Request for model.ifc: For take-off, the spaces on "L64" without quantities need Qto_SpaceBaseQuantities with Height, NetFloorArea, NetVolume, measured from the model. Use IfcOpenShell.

First a look at what the model holds.

```python
import ifcopenshell
import ifcopenshell.util.element
import ifcopenshell.util.unit

model = ifcopenshell.open("model.ifc")
print(model.schema)
for unit_type in ("LENGTHUNIT", "AREAUNIT", "VOLUMEUNIT"):
    print(unit_type, ifcopenshell.util.unit.calculate_unit_scale(model, unit_type))
storey = next(s for s in model.by_type("IfcBuildingStorey") if s.Name == "L64")
spaces = [e for e in ifcopenshell.util.element.get_decomposition(storey) if e.is_a("IfcSpace")]
for e in sorted(spaces, key=lambda e: e.id()):
    print(e.id(), e.is_a(), e.Name, list(ifcopenshell.util.element.get_psets(e, qtos_only=True)), sep=" | ")
```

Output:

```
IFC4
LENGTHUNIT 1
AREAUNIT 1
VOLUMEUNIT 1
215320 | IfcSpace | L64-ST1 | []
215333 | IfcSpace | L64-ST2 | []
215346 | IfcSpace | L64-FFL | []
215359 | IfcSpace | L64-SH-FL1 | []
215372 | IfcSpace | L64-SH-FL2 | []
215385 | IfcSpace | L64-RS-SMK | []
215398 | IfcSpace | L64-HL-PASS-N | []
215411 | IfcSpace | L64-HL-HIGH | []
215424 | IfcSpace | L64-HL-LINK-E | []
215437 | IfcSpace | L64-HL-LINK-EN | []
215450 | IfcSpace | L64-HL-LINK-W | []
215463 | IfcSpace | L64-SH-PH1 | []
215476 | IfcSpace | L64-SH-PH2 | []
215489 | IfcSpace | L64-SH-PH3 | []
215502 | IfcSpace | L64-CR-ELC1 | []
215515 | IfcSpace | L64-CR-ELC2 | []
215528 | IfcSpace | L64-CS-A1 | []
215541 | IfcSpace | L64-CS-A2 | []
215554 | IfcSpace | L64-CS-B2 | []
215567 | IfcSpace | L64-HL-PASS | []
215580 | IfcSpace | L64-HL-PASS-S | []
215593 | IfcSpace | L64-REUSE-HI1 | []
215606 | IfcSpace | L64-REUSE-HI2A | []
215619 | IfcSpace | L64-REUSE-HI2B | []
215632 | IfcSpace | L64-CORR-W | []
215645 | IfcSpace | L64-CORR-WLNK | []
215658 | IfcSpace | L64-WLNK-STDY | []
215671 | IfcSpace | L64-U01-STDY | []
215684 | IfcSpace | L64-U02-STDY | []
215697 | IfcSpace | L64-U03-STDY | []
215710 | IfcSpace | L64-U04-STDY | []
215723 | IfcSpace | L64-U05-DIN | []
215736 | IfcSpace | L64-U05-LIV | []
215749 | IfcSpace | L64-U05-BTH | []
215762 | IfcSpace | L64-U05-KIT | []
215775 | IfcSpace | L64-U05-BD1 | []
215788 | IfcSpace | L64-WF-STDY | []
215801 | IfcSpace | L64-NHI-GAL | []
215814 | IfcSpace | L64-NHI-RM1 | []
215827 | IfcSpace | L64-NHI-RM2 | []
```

```python
import ifcopenshell
import ifcopenshell.api.pset
import ifcopenshell.geom
import ifcopenshell.util.element
import ifcopenshell.util.shape
import ifcopenshell.util.unit

model = ifcopenshell.open("model.ifc")
unit_scale = ifcopenshell.util.unit.calculate_unit_scale(model)
area_scale = ifcopenshell.util.unit.calculate_unit_scale(model, "AREAUNIT")
volume_scale = ifcopenshell.util.unit.calculate_unit_scale(model, "VOLUMEUNIT")
settings = ifcopenshell.geom.settings()

storey = next(s for s in model.by_type("IfcBuildingStorey") if s.Name == "L64")
spaces = [e for e in ifcopenshell.util.element.get_decomposition(storey) if e.is_a("IfcSpace")]

for e in sorted(spaces, key=lambda e: e.id()):
    if ifcopenshell.util.element.get_psets(e, qtos_only=True, should_inherit=False):
        continue
    # Geometry comes back in metres, in the element's own axes.
    shape = ifcopenshell.geom.create_shape(settings, e)
    values = {
        "Height": ifcopenshell.util.shape.get_z(shape.geometry) / unit_scale,
        "NetFloorArea": ifcopenshell.util.shape.get_footprint_area(shape.geometry) / area_scale,
        "NetVolume": ifcopenshell.util.shape.get_volume(shape.geometry) / volume_scale,
    }
    qto = ifcopenshell.api.pset.add_qto(model, product=e, name="Qto_SpaceBaseQuantities")
    ifcopenshell.api.pset.edit_qto(model, qto=qto, properties=values)
    print(e.id(), {k: round(v, 3) for k, v in values.items()})

model.write("model-out.ifc")
```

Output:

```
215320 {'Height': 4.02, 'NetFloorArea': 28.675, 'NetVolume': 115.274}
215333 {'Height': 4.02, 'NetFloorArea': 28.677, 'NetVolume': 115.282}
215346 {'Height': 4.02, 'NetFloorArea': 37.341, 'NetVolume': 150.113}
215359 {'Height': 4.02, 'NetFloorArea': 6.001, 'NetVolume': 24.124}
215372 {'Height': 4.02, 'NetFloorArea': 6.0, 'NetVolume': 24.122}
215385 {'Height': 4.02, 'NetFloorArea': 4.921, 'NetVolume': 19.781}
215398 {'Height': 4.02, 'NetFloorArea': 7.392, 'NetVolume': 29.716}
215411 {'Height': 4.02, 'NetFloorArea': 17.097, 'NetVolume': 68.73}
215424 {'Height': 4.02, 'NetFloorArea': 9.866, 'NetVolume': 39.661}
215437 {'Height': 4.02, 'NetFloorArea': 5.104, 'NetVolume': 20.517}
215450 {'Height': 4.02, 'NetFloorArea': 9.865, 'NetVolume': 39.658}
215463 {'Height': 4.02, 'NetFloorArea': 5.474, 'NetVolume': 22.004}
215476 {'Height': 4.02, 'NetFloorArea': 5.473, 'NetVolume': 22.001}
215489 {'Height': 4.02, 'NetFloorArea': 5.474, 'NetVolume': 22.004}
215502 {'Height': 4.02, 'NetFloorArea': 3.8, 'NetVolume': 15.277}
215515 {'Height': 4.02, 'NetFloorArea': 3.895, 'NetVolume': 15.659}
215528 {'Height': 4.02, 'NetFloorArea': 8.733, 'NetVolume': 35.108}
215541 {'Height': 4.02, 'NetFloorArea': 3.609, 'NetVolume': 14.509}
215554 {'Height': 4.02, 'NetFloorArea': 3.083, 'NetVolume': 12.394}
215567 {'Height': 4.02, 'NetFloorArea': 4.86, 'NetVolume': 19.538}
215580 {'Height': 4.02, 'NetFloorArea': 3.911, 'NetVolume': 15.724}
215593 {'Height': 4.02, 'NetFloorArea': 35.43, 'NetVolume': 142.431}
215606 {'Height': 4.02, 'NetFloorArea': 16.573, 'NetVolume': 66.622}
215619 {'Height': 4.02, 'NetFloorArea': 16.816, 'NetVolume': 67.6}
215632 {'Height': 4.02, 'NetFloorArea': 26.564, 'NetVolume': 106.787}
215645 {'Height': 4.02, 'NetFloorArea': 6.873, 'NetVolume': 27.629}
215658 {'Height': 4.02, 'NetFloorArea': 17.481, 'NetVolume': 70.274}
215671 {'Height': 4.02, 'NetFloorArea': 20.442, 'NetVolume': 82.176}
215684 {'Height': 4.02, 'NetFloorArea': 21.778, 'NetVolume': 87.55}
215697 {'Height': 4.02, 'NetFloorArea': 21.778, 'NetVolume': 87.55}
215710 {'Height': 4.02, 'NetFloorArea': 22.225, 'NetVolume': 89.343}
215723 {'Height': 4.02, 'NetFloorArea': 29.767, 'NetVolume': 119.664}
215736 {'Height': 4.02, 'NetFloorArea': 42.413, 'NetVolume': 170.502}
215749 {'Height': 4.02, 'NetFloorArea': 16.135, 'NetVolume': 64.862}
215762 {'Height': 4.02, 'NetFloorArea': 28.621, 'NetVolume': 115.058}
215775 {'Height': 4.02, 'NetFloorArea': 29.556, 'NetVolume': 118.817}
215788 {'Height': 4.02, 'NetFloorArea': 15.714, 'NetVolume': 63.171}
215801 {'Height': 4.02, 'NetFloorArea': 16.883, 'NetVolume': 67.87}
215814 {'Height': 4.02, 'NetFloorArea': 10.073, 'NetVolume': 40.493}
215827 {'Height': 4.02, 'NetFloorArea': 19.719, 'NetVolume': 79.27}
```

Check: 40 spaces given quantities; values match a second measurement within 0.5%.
